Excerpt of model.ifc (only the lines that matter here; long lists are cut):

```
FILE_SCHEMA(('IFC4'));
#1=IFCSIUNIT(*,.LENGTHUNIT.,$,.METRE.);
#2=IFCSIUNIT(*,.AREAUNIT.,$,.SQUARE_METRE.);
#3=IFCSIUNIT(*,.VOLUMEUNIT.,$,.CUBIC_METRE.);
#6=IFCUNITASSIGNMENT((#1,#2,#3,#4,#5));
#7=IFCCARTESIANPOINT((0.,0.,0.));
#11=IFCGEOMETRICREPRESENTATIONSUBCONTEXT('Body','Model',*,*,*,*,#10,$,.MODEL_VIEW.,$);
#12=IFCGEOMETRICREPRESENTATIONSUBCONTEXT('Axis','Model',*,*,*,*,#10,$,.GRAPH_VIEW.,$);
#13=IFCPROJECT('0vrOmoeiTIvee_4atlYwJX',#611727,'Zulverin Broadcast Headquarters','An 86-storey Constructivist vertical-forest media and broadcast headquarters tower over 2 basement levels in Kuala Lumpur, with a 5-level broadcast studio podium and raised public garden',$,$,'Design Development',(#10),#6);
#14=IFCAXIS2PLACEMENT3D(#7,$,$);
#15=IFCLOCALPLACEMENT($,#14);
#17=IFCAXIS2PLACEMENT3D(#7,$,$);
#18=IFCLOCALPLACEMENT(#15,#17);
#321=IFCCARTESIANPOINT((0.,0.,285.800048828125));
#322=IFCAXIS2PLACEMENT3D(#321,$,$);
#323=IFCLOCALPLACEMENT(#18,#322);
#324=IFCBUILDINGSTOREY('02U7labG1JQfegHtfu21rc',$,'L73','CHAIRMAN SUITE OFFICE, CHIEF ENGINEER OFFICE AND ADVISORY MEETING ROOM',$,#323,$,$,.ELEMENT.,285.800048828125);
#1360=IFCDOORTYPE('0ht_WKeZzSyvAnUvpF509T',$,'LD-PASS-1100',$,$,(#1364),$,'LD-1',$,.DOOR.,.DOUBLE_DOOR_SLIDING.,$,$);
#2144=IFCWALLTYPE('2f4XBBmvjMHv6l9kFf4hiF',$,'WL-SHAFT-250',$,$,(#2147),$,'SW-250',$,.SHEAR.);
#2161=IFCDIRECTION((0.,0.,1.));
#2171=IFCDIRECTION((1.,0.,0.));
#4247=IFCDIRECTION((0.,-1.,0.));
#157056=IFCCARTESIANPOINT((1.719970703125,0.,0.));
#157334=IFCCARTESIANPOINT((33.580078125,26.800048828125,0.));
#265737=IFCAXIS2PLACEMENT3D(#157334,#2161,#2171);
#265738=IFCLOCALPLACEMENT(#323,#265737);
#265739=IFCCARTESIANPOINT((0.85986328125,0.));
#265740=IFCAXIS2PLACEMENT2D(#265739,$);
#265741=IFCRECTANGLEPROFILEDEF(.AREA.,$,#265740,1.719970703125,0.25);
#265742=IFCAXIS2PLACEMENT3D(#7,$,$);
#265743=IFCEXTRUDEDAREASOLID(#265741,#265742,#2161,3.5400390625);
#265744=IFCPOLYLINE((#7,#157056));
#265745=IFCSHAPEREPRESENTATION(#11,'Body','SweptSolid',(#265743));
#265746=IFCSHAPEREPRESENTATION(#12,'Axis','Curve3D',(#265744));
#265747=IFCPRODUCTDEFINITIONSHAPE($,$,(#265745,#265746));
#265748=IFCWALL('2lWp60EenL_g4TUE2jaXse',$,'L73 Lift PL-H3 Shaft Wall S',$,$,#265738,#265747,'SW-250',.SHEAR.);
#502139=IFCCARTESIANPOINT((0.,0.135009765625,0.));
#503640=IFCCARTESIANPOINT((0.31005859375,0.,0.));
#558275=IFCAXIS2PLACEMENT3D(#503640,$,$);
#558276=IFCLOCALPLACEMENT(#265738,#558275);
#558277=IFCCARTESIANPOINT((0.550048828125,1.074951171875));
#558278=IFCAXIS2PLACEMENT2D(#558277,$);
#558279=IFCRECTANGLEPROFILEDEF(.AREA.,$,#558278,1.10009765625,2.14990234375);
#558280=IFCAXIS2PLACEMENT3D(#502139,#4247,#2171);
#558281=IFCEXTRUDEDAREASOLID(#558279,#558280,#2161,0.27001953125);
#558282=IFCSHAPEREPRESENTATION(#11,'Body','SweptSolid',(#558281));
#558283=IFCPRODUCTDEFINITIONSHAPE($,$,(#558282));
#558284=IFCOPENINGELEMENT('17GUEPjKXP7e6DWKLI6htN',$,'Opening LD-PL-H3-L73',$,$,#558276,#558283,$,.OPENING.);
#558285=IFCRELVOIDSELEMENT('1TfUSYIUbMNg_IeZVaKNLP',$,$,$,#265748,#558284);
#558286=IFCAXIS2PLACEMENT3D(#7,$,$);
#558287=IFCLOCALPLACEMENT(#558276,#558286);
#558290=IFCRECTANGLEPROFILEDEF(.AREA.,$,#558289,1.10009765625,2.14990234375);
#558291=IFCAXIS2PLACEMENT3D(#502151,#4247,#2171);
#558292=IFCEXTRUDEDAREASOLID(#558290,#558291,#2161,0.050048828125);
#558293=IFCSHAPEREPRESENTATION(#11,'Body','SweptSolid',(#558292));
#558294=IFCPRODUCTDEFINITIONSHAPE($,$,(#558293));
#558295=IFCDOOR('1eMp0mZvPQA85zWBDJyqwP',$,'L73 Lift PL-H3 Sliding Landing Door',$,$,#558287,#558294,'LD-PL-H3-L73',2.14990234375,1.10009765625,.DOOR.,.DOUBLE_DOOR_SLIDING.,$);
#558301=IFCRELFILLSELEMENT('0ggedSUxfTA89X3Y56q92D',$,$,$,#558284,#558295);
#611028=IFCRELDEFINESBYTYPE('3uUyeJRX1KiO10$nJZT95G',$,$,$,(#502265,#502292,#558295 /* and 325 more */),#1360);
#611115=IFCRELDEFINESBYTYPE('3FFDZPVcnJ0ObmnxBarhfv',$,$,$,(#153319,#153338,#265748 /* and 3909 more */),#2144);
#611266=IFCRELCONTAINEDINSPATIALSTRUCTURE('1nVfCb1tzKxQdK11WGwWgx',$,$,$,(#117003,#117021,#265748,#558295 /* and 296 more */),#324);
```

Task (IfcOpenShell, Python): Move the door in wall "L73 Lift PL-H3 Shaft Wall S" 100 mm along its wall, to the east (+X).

```python
import ifcopenshell
import ifcopenshell.api.geometry
import ifcopenshell.util.placement

model = ifcopenshell.open("model.ifc")

door = model.by_id(558295)
opening = door.FillsVoids[0].RelatingOpeningElement
wall = opening.VoidsElements[0].RelatingBuildingElement

wall_matrix = ifcopenshell.util.placement.get_local_placement(wall.ObjectPlacement)
shift = wall_matrix[:3, 0] * 0.1
before = ifcopenshell.util.placement.get_local_placement(door.ObjectPlacement)[:3, 3].copy()

# The door is placed relative to its opening, so it follows when the opening moves.
matrix = ifcopenshell.util.placement.get_local_placement(opening.ObjectPlacement)
matrix[:3, 3] += shift
ifcopenshell.api.geometry.edit_object_placement(
    model, product=opening, matrix=matrix, is_si=False, should_transform_children=True
)

after = ifcopenshell.util.placement.get_local_placement(door.ObjectPlacement)[:3, 3]
print("door moved by", (after - before).round(3) + 0.0)

model.write("model_updated.ifc")
```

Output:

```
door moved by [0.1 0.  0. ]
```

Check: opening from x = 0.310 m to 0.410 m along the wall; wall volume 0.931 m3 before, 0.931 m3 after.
